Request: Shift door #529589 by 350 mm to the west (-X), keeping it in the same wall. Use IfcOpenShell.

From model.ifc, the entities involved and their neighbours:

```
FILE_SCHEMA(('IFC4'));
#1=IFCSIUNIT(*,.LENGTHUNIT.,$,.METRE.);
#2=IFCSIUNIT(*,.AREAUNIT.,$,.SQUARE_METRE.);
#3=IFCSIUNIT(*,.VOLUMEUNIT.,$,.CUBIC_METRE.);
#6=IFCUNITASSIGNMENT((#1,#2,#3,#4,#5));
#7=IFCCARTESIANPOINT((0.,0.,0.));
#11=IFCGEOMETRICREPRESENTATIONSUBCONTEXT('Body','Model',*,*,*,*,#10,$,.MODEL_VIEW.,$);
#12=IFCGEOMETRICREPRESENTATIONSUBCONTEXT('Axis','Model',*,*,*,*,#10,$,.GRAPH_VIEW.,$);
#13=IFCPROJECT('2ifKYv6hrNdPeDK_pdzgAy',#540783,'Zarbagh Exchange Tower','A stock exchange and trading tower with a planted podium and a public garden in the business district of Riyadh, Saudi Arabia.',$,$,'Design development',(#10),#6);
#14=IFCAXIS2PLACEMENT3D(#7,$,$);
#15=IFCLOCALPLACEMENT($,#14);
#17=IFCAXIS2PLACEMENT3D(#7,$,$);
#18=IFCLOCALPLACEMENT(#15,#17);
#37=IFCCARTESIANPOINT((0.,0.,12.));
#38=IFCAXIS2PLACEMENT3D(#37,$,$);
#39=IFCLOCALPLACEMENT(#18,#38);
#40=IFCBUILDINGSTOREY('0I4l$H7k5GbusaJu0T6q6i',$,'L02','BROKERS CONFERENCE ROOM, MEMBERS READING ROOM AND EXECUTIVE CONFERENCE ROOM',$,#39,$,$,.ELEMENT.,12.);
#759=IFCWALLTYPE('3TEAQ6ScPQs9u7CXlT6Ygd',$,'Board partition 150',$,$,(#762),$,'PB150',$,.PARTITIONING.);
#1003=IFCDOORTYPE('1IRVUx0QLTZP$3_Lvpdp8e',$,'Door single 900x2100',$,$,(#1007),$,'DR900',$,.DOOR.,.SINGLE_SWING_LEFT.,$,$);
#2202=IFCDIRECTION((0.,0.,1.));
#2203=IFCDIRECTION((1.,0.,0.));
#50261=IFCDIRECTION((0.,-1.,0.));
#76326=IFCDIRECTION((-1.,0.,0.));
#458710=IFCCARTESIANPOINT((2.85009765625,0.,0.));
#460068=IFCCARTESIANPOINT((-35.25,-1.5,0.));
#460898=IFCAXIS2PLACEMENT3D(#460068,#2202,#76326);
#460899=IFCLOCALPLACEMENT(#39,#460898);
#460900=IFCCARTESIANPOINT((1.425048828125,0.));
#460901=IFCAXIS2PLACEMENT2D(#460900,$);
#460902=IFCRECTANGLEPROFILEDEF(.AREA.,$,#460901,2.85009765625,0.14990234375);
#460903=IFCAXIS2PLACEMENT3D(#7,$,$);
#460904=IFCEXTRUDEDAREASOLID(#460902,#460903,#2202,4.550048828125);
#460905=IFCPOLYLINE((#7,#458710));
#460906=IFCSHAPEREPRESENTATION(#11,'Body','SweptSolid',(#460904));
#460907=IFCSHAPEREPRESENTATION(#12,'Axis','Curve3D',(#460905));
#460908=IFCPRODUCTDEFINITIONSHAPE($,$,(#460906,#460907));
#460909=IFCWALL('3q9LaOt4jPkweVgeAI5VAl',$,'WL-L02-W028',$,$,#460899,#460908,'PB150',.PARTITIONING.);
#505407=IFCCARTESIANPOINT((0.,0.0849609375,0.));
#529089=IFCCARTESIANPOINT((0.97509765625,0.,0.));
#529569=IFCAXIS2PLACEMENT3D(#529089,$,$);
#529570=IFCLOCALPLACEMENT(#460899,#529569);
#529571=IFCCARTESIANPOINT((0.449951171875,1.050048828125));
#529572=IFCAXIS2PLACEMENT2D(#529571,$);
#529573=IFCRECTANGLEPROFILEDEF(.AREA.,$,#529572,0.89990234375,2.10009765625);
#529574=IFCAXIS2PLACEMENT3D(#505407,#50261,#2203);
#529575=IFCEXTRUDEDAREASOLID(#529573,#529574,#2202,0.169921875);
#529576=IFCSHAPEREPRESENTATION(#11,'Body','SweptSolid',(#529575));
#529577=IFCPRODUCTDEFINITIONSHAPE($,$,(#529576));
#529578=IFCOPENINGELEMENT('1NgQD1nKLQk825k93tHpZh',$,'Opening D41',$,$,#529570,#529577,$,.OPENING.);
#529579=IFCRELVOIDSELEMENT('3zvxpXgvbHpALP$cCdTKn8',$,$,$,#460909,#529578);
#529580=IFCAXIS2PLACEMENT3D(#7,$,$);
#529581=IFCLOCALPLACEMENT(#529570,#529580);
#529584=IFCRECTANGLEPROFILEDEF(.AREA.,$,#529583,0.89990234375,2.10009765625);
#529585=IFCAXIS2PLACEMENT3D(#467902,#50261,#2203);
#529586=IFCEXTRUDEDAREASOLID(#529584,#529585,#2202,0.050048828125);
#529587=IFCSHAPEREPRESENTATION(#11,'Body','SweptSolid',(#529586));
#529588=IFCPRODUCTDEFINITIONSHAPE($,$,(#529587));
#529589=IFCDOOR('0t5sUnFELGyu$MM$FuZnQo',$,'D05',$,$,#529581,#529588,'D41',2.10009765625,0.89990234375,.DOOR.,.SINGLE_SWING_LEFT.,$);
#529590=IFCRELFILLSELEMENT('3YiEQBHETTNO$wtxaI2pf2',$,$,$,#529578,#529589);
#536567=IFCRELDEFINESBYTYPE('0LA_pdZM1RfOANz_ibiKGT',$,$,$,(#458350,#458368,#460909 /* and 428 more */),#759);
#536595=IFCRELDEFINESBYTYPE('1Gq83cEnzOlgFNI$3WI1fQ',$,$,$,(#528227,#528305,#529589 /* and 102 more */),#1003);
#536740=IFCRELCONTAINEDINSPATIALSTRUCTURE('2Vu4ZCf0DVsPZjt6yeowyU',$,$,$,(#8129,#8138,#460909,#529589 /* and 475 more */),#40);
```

```python
import ifcopenshell
import ifcopenshell.api.geometry
import ifcopenshell.util.placement
import ifcopenshell.util.unit

model = ifcopenshell.open("model.ifc")
unit_scale = ifcopenshell.util.unit.calculate_unit_scale(model)

door = model.by_id(529589)
opening = door.FillsVoids[0].RelatingOpeningElement
wall = opening.VoidsElements[0].RelatingBuildingElement

wall_matrix = ifcopenshell.util.placement.get_local_placement(wall.ObjectPlacement)
shift = wall_matrix[:3, 0] * 0.35 / unit_scale
before = ifcopenshell.util.placement.get_local_placement(door.ObjectPlacement)[:3, 3].copy()

# The door is placed relative to its opening, so it follows when the opening moves.
matrix = ifcopenshell.util.placement.get_local_placement(opening.ObjectPlacement)
matrix[:3, 3] += shift
ifcopenshell.api.geometry.edit_object_placement(
    model, product=opening, matrix=matrix, is_si=False, should_transform_children=True
)

after = ifcopenshell.util.placement.get_local_placement(door.ObjectPlacement)[:3, 3]
print("door moved by", (after - before).round(3) + 0.0)

model.write("model_rev.ifc")
```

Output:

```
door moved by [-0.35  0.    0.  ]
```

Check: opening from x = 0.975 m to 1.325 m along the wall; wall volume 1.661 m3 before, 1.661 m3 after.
